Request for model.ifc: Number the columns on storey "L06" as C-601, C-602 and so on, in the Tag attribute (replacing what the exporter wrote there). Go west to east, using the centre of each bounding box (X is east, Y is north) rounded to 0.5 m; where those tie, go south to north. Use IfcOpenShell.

First a look at what the model holds.

```python
import ifcopenshell
import ifcopenshell.util.element
import ifcopenshell.util.placement

model = ifcopenshell.open("model.ifc")
print(model.schema)
storey = next(s for s in model.by_type("IfcBuildingStorey") if s.Name == "L06")
columns = [e for e in ifcopenshell.util.element.get_decomposition(storey) if e.is_a("IfcColumn")]
for e in sorted(columns, key=lambda e: e.id()):
    origin = ifcopenshell.util.placement.get_local_placement(e.ObjectPlacement)[:3, 3]
    print(e.id(), e.Tag, e.Name, origin.round(2) + 0.0, sep=" | ")
```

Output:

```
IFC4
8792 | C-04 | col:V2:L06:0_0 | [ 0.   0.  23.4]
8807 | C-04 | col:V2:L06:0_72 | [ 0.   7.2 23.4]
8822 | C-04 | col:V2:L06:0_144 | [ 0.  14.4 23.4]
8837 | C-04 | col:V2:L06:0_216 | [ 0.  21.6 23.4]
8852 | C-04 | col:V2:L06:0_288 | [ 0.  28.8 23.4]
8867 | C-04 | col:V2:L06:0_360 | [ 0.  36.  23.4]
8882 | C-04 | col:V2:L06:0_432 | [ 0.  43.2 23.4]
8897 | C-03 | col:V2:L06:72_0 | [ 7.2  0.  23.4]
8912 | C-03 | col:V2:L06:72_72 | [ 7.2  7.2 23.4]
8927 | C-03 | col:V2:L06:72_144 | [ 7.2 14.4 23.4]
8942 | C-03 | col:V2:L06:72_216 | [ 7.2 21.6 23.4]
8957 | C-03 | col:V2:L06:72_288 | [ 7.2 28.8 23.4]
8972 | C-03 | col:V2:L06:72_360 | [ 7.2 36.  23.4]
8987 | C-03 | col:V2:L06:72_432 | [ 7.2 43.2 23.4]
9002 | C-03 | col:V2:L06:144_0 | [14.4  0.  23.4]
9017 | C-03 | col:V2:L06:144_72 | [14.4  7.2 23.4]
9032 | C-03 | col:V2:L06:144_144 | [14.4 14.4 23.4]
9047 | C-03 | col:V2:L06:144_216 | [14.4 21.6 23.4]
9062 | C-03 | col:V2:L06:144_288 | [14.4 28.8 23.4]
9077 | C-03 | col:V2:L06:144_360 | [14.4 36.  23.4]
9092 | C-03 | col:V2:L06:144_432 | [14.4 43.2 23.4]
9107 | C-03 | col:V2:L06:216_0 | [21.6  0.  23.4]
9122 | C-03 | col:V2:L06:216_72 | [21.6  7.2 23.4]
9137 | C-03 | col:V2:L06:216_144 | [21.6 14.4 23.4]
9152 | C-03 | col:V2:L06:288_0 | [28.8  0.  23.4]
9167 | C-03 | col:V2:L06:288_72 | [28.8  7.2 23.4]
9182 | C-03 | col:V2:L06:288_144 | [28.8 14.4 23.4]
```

```python
import ifcopenshell
import ifcopenshell.geom
import ifcopenshell.util.element
import ifcopenshell.util.shape

model = ifcopenshell.open("model.ifc")
settings = ifcopenshell.geom.settings()
settings.set("use-world-coords", True)


def centre(element):
    shape = ifcopenshell.geom.create_shape(settings, element)
    return ifcopenshell.util.shape.get_bbox_centroid(shape.geometry)


storey = next(s for s in model.by_type("IfcBuildingStorey") if s.Name == "L06")
columns = [e for e in ifcopenshell.util.element.get_decomposition(storey) if e.is_a("IfcColumn")]

# Insertion points can sit at a corner or the storey origin, so sort by the geometry (in metres).
centres = {e: centre(e) for e in columns}
columns.sort(key=lambda e: (round(centres[e][0] / 0.5), centres[e][1]))

for i, e in enumerate(columns, start=1):
    number = f"C-6{i:02d}"
    e.Tag = number
    print(e.id(), number)

model.write("model_edited.ifc")
```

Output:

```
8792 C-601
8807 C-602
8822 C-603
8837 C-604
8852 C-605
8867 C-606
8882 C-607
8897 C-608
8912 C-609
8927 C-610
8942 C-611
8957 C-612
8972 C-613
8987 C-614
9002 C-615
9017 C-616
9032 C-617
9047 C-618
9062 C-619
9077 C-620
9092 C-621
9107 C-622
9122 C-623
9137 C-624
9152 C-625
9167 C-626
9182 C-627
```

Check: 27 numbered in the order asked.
